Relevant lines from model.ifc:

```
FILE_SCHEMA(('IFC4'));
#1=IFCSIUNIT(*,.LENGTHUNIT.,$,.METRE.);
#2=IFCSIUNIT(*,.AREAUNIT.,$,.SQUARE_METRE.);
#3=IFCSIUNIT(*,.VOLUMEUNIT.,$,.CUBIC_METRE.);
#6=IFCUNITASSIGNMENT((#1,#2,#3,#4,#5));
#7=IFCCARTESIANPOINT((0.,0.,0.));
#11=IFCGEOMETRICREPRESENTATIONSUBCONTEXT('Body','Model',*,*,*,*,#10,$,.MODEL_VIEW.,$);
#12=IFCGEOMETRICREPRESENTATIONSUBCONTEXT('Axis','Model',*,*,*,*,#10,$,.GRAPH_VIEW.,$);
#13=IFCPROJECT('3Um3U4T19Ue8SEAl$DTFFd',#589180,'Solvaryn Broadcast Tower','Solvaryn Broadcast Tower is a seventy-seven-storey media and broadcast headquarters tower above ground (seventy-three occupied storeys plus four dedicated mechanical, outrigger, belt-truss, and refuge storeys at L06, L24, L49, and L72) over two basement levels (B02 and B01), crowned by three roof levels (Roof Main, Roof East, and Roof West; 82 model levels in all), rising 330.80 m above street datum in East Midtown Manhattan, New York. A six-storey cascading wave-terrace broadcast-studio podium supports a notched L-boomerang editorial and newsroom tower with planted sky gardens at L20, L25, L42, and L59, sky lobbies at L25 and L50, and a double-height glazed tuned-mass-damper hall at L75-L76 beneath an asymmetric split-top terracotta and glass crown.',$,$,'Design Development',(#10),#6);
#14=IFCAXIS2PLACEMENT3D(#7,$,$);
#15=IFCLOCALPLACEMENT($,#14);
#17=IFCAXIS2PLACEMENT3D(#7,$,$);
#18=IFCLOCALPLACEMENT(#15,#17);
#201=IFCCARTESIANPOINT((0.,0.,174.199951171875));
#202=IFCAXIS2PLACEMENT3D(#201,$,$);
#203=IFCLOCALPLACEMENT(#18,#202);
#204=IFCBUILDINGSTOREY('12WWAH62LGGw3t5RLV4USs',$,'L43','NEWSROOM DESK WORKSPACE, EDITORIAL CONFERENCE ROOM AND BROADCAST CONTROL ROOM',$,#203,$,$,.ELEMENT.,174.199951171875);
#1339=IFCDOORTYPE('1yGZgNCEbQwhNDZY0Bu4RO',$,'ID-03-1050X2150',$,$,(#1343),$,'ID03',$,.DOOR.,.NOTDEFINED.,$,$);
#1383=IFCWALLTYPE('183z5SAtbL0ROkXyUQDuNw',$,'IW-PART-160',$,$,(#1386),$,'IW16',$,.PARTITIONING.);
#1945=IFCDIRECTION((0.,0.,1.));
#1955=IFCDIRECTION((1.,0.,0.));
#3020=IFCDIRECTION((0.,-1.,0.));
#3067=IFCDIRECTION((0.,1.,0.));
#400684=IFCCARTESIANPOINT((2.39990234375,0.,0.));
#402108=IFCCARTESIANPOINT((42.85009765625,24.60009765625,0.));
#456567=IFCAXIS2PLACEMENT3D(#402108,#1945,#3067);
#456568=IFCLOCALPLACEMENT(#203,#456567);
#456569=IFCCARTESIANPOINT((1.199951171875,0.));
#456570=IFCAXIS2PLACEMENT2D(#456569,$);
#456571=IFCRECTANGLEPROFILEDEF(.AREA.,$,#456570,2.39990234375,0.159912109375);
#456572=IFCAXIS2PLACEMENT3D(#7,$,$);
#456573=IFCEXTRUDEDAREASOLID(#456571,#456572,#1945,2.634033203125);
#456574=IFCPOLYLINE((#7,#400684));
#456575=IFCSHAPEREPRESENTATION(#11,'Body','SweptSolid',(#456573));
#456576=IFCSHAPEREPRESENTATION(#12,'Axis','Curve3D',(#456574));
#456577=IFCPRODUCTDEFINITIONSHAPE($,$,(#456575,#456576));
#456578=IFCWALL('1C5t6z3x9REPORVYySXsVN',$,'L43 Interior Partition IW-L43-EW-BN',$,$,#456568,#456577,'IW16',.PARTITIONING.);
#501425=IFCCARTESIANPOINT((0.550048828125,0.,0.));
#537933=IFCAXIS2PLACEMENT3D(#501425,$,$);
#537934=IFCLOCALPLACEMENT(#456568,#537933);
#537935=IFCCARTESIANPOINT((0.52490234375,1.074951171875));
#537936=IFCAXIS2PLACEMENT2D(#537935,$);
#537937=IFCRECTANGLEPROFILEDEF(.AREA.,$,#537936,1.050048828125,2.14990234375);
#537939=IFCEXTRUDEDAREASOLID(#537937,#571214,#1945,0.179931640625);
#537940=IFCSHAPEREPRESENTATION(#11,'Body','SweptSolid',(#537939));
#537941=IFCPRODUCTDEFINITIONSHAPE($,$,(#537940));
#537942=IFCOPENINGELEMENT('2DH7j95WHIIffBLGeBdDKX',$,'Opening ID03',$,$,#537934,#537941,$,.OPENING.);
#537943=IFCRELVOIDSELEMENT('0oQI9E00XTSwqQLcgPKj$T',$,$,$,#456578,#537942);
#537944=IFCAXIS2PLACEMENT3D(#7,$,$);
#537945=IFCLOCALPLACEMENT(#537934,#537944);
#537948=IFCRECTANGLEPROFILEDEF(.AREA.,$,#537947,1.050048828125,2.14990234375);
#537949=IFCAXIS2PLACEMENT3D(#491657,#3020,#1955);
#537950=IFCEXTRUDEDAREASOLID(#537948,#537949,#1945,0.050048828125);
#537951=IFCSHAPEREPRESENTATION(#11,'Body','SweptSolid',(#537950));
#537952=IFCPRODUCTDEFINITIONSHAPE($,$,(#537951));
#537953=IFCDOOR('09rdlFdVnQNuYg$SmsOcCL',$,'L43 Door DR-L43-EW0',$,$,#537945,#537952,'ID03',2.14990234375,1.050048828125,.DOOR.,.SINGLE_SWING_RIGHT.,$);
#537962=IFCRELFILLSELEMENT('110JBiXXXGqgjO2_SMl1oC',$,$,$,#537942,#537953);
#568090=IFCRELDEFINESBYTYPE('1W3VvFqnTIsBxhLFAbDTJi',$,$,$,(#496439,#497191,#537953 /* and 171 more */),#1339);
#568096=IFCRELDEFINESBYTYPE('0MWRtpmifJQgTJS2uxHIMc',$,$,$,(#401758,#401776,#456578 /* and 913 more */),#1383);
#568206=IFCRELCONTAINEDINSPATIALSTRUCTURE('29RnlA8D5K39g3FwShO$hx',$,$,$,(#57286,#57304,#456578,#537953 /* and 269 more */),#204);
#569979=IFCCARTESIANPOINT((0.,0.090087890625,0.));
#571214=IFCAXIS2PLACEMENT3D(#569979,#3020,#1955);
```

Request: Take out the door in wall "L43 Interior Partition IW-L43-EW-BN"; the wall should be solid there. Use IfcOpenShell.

```python
import ifcopenshell
import ifcopenshell.api.feature
import ifcopenshell.api.root
import ifcopenshell.geom
import ifcopenshell.util.shape

model = ifcopenshell.open("model.ifc")
settings = ifcopenshell.geom.settings()


def volume(element):
    """Net volume in cubic metres, openings subtracted."""
    shape = ifcopenshell.geom.create_shape(settings, element)
    return ifcopenshell.util.shape.get_volume(shape.geometry)


door = model.by_guid("09rdlFdVnQNuYg$SmsOcCL")
opening = door.FillsVoids[0].RelatingOpeningElement
wall = opening.VoidsElements[0].RelatingBuildingElement
before = volume(wall)

ifcopenshell.api.root.remove_product(model, product=door)
ifcopenshell.api.feature.remove_feature(model, feature=opening)

after = volume(wall)

print(f"wall volume {before:.3f} -> {after:.3f} m3")

model.write("model_updated.ifc")
```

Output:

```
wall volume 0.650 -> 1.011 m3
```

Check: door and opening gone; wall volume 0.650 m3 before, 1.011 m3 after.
